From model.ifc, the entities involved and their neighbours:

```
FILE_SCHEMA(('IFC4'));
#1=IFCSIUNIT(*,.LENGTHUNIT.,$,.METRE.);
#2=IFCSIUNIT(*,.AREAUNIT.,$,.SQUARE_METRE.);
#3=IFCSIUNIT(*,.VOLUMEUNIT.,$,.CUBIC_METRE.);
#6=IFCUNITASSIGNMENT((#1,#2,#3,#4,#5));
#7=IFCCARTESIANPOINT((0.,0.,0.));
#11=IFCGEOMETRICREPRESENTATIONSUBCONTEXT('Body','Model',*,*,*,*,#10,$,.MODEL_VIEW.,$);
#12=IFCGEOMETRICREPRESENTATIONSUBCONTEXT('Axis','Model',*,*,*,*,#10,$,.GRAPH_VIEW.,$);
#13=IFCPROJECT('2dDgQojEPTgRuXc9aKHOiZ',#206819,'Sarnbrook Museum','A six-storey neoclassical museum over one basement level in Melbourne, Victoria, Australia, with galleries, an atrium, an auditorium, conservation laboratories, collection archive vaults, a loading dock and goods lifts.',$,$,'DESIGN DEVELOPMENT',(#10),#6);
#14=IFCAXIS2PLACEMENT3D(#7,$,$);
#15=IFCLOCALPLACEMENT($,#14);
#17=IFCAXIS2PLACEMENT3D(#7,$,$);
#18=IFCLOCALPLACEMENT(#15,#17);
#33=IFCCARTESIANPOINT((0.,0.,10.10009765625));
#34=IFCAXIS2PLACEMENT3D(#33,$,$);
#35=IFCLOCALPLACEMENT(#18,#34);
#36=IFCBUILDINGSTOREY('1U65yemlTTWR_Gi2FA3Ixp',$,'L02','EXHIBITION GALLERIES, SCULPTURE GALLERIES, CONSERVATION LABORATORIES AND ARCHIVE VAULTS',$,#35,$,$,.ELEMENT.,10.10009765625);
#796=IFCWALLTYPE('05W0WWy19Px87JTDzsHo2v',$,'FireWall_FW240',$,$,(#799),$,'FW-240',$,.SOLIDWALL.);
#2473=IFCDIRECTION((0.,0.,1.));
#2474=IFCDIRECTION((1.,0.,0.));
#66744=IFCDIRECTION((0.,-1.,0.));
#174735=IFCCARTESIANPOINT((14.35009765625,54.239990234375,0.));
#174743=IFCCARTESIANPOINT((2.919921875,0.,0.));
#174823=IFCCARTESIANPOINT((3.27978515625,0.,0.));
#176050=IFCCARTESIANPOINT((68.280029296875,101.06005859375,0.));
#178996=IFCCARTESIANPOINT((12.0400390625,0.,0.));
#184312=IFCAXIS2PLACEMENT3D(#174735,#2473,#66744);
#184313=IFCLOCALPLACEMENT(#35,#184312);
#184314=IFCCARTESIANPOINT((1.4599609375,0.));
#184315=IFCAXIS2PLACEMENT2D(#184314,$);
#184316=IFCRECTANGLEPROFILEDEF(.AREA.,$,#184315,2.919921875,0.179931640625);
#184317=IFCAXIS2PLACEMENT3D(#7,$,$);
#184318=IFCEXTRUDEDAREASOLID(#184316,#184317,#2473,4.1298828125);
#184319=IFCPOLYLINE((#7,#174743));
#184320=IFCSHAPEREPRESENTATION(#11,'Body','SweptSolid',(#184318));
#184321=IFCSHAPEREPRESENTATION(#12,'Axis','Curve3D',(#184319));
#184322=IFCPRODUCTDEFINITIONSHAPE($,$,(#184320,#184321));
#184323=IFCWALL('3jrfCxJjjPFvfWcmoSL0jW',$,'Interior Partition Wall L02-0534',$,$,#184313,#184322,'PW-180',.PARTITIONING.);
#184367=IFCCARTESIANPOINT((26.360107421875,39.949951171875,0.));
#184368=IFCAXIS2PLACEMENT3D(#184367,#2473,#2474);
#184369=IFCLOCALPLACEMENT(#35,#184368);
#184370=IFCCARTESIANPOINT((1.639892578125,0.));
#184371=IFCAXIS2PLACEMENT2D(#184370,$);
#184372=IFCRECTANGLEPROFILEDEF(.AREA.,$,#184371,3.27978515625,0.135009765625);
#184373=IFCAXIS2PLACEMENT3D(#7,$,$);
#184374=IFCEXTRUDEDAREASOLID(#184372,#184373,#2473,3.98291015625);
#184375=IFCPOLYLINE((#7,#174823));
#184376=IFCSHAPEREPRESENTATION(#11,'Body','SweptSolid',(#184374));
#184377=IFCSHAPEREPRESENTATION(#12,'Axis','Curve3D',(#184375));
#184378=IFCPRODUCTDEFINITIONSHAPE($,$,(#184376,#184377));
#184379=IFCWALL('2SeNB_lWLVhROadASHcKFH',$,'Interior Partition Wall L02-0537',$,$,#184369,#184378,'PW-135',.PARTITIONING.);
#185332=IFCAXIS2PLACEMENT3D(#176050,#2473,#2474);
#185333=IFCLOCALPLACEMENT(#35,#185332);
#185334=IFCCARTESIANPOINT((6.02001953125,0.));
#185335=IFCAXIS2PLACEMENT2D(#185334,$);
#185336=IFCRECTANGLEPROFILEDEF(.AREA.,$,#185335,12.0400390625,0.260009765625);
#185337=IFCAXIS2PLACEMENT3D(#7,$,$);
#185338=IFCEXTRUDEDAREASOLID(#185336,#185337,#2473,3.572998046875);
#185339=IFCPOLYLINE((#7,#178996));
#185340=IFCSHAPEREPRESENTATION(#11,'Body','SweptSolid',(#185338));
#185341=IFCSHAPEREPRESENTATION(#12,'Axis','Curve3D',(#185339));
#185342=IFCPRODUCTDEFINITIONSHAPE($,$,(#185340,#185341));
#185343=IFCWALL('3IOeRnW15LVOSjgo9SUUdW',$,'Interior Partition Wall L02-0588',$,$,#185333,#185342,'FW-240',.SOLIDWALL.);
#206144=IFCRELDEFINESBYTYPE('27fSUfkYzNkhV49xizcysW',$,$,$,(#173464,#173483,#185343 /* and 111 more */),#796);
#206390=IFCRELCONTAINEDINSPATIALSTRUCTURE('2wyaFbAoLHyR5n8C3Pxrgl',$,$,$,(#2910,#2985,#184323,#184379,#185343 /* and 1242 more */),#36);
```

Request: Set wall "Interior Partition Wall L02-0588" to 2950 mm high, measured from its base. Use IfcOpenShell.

```python
import ifcopenshell
import ifcopenshell.geom
import ifcopenshell.util.representation
import ifcopenshell.util.shape
import ifcopenshell.util.unit

model = ifcopenshell.open("model.ifc")
unit_scale = ifcopenshell.util.unit.calculate_unit_scale(model)
settings = ifcopenshell.geom.settings()


def volume(element):
    """Net volume in cubic metres, openings subtracted."""
    shape = ifcopenshell.geom.create_shape(settings, element)
    return ifcopenshell.util.shape.get_volume(shape.geometry)


wall = model.by_guid("3IOeRnW15LVOSjgo9SUUdW")
before = volume(wall)

body = ifcopenshell.util.representation.get_representation(wall, "Model", "Body")
solid = body.Items[0]
old_height = solid.Depth
solid.Depth = 2.95 / unit_scale
after = volume(wall)

print(f"height {old_height:g} -> {solid.Depth:g}, volume {before:.3f} -> {after:.3f} m3")

model.write("model_v2.ifc")
```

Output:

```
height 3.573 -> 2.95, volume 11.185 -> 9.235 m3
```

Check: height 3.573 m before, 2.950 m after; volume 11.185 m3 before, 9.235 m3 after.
